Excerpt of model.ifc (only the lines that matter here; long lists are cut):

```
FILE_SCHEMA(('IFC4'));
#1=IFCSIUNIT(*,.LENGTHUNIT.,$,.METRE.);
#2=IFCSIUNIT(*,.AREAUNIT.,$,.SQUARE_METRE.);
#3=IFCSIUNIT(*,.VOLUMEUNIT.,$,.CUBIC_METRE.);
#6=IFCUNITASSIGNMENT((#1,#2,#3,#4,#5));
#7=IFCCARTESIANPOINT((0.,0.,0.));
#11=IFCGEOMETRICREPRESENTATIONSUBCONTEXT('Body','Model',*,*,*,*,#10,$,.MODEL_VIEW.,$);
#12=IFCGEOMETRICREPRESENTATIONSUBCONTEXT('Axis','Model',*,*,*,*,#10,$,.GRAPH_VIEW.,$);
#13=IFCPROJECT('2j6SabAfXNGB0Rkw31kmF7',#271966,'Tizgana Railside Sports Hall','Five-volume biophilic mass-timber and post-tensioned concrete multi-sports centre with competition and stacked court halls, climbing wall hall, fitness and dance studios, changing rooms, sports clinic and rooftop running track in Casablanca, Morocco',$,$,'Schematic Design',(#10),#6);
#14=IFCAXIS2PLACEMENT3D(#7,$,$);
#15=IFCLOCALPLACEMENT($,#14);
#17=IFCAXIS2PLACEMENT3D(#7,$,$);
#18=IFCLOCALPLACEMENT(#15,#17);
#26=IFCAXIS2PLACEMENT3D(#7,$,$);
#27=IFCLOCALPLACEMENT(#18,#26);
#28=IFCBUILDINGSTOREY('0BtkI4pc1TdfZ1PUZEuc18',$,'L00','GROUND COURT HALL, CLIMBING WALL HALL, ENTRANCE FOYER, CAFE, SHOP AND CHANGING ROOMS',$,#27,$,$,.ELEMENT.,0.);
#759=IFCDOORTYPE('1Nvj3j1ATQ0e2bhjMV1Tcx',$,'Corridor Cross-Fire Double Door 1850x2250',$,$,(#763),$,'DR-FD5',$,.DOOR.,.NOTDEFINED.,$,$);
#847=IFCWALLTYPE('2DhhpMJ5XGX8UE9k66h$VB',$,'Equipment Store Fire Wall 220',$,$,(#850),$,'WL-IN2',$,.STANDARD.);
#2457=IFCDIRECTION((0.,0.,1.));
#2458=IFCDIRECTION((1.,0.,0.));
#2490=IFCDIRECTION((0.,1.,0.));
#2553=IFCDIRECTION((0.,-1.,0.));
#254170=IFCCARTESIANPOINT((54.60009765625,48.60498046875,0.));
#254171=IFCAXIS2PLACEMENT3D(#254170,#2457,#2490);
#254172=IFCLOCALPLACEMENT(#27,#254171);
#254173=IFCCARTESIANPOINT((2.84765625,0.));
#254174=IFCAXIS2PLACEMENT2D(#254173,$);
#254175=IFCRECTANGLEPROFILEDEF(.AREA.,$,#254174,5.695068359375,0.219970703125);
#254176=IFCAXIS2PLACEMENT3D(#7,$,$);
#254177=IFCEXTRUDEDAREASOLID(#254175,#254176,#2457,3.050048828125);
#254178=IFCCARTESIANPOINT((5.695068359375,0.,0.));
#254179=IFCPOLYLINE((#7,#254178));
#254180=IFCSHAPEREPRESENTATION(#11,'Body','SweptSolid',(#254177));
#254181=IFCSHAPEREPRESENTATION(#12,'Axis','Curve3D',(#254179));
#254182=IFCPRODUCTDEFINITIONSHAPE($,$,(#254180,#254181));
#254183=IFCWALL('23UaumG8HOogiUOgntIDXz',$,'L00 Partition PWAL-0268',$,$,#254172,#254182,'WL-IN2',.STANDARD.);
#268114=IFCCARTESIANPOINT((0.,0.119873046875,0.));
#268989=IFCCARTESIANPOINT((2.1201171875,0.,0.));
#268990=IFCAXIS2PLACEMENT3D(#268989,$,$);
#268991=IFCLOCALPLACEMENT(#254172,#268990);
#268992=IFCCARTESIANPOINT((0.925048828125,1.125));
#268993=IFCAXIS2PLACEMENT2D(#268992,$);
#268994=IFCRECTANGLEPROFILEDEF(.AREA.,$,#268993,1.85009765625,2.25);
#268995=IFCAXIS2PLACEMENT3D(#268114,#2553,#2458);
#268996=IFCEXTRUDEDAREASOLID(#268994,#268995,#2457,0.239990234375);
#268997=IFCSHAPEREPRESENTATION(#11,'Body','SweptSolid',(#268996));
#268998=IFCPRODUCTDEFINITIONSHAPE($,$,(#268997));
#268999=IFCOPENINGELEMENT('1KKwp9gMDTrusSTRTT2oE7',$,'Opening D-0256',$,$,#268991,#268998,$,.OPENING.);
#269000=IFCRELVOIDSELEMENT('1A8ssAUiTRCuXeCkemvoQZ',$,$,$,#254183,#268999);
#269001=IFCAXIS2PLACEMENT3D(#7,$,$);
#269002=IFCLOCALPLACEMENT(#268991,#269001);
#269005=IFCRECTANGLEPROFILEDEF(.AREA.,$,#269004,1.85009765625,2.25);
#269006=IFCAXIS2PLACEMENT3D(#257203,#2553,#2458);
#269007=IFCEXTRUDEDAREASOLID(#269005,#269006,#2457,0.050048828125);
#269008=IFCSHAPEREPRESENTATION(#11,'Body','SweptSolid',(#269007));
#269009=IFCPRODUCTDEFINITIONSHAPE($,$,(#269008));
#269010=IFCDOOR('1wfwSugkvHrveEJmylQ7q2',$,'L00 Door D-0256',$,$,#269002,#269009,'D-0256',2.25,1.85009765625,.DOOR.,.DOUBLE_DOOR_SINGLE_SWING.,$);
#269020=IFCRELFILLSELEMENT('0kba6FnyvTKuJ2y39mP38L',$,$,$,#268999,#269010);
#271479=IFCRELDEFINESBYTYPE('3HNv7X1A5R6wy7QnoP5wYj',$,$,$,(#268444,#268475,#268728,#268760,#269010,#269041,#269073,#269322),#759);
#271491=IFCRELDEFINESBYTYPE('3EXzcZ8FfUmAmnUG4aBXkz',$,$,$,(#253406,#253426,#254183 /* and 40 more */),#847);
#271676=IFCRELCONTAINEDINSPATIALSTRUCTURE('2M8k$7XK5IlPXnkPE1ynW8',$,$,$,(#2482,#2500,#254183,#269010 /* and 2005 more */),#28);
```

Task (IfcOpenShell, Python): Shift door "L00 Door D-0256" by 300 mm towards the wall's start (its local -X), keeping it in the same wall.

```python
import ifcopenshell
import ifcopenshell.api.geometry
import ifcopenshell.util.placement

model = ifcopenshell.open("model.ifc")

door = model.by_id(269010)
opening = door.FillsVoids[0].RelatingOpeningElement
wall = opening.VoidsElements[0].RelatingBuildingElement

wall_matrix = ifcopenshell.util.placement.get_local_placement(wall.ObjectPlacement)
shift = wall_matrix[:3, 0] * -0.3
before = ifcopenshell.util.placement.get_local_placement(door.ObjectPlacement)[:3, 3].copy()

# The door is placed relative to its opening, so it follows when the opening moves.
matrix = ifcopenshell.util.placement.get_local_placement(opening.ObjectPlacement)
matrix[:3, 3] += shift
ifcopenshell.api.geometry.edit_object_placement(
    model, product=opening, matrix=matrix, is_si=False, should_transform_children=True
)

after = ifcopenshell.util.placement.get_local_placement(door.ObjectPlacement)[:3, 3]
print("door moved by", (after - before).round(3) + 0.0)

model.write("model_v2.ifc")
```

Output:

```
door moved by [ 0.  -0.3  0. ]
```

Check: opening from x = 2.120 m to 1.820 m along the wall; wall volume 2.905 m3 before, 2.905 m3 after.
